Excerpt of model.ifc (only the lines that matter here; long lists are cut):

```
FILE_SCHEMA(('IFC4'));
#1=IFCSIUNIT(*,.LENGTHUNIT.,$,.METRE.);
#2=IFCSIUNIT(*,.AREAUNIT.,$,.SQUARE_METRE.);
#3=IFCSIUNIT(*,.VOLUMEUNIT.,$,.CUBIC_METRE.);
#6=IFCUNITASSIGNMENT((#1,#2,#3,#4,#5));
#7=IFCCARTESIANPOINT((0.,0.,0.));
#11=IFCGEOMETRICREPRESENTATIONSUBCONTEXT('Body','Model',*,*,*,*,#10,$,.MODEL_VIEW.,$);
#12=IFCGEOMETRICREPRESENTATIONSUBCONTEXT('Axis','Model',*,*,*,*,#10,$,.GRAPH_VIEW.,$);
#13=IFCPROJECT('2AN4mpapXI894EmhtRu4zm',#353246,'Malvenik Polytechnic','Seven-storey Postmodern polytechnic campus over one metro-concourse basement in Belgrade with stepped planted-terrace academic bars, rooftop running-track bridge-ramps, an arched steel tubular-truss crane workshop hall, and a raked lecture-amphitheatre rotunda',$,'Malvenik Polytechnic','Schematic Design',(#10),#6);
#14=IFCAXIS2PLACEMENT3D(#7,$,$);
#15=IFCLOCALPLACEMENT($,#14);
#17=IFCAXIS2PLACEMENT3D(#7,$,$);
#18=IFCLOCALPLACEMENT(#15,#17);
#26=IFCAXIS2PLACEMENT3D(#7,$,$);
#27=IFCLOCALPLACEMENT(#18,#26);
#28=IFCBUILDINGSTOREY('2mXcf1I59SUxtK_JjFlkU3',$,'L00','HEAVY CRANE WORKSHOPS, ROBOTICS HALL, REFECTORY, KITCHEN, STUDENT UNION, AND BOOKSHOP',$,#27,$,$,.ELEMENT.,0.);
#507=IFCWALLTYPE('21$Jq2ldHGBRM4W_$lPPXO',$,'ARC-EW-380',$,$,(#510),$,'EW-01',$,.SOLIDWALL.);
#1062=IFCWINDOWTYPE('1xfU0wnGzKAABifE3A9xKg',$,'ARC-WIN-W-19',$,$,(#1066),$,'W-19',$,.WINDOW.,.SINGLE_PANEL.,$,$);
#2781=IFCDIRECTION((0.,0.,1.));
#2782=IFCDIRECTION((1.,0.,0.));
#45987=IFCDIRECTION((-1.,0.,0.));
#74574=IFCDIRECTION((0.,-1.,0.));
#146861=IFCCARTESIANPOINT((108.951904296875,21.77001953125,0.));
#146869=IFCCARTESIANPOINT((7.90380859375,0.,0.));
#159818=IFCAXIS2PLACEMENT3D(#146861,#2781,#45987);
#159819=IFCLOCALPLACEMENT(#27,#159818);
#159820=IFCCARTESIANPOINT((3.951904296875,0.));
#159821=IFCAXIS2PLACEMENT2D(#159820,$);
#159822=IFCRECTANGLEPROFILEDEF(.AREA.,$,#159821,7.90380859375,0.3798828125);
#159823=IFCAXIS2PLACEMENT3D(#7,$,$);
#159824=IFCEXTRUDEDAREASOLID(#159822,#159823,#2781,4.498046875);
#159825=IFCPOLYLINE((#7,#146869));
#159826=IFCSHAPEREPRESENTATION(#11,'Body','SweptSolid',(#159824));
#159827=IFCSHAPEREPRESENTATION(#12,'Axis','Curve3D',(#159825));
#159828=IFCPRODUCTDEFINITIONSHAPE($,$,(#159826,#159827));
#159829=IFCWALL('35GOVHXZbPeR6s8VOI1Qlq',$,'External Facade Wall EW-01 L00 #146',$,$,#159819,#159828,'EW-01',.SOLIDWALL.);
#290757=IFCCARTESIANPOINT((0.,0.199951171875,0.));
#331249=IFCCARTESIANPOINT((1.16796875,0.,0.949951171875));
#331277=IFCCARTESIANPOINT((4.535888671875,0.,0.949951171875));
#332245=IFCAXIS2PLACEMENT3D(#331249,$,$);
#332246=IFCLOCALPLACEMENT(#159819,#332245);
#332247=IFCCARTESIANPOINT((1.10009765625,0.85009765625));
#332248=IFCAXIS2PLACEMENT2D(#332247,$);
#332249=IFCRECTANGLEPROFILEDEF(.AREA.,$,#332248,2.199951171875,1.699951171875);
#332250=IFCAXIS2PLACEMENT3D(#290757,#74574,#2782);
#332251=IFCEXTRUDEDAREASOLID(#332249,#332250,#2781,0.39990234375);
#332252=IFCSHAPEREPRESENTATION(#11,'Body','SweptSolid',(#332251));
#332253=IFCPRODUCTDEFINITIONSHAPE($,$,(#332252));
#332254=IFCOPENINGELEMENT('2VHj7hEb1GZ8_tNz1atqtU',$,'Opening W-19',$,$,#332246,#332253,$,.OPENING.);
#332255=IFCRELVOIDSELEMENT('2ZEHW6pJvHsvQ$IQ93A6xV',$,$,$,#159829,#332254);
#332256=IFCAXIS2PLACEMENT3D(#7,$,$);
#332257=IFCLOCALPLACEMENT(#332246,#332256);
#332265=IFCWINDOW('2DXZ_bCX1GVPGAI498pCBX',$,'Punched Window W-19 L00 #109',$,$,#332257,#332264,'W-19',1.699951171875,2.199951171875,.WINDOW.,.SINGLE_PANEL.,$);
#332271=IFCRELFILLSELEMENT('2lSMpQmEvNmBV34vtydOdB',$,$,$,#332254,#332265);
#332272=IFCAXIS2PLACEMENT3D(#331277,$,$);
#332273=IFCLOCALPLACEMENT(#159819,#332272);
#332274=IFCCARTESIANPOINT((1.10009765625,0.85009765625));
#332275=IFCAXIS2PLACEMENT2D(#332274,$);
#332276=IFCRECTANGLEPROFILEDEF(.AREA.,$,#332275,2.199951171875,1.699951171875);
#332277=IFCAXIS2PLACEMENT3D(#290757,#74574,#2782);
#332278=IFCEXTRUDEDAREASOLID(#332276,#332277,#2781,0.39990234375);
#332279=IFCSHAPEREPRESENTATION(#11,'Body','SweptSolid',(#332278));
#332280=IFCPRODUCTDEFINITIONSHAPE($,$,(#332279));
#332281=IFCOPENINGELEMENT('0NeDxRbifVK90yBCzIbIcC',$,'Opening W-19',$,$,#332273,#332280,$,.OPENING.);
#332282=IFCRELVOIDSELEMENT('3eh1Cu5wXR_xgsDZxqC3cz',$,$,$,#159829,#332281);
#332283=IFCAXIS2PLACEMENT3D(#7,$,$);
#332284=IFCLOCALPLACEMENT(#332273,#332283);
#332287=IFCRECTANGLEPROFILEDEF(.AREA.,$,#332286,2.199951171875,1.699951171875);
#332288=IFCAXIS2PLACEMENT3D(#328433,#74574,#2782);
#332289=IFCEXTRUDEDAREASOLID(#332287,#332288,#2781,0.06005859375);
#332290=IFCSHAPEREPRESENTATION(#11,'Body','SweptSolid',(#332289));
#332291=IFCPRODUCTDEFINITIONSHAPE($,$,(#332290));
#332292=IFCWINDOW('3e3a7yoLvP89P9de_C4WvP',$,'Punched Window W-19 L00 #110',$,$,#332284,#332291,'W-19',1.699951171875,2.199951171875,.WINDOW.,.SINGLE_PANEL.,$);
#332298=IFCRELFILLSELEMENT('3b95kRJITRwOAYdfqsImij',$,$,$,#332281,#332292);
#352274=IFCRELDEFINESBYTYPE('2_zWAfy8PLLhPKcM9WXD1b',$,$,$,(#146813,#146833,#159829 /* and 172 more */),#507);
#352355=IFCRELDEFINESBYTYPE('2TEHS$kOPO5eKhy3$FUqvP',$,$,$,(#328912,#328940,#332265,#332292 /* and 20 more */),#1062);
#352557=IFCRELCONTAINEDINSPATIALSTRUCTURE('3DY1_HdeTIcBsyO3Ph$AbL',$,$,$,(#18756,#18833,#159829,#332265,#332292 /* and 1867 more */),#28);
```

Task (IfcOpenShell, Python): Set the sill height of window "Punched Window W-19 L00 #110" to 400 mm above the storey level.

```python
import numpy as np
import ifcopenshell
import ifcopenshell.api.geometry
import ifcopenshell.geom
import ifcopenshell.util.element
import ifcopenshell.util.placement
import ifcopenshell.util.shape
import ifcopenshell.util.unit

model = ifcopenshell.open("model.ifc")
unit_scale = ifcopenshell.util.unit.calculate_unit_scale(model)

window = model.by_id(332292)
opening = window.FillsVoids[0].RelatingOpeningElement
storey = ifcopenshell.util.element.get_container(window, ifc_class="IfcBuildingStorey")
level = ifcopenshell.util.placement.get_local_placement(storey.ObjectPlacement)[2, 3]

# The opening's origin need not be at the sill, so measure its lowest point.
shape = ifcopenshell.geom.create_shape(ifcopenshell.geom.settings(), opening)
bottom = ifcopenshell.util.shape.get_shape_bottom_elevation(shape, shape.geometry) / unit_scale
dz = level + 0.4 / unit_scale - bottom

shift = np.array([0.0, 0.0, dz])
# The window is placed relative to its opening, so it follows when the opening moves.
matrix = ifcopenshell.util.placement.get_local_placement(opening.ObjectPlacement)
matrix[:3, 3] += shift
ifcopenshell.api.geometry.edit_object_placement(
    model, product=opening, matrix=matrix, is_si=False, should_transform_children=True
)

print(f"moved by {dz * unit_scale:+.3f} m")

model.write("model_v2.ifc")
```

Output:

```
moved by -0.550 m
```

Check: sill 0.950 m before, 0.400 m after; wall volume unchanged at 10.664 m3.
